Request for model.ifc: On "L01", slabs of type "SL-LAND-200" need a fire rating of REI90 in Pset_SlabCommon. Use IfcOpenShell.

First a look at what the model holds.

```python
import ifcopenshell
import ifcopenshell.util.element

model = ifcopenshell.open("model.ifc")
print(model.schema)
storey = next(s for s in model.by_type("IfcBuildingStorey") if s.Name == "L01")
slabs = [e for e in ifcopenshell.util.element.get_decomposition(storey) if e.is_a("IfcSlab")]
seen = {}
for e in slabs:
    element_type = ifcopenshell.util.element.get_type(e)
    key = (element_type.Name if element_type != e and element_type else None, ifcopenshell.util.element.get_pset(e, "Pset_SlabCommon", "FireRating"))
    seen[key] = seen.get(key, 0) + 1
for (name, value), count in sorted(seen.items(), key=str):
    print(count, "x", name, "|", value)
```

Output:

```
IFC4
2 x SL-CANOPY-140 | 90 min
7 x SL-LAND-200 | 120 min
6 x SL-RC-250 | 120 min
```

```python
import ifcopenshell
import ifcopenshell.api.pset
import ifcopenshell.util.element

model = ifcopenshell.open("model.ifc")

storey = next(s for s in model.by_type("IfcBuildingStorey") if s.Name == "L01")
slabs = [e for e in ifcopenshell.util.element.get_decomposition(storey) if e.is_a("IfcSlab")]

count = 0
for e in slabs:
    element_type = ifcopenshell.util.element.get_type(e)
    if element_type in (None, e) or element_type.Name != "SL-LAND-200":
        continue
    # add_pset returns the element's existing set when there is one.
    pset = ifcopenshell.api.pset.add_pset(model, product=e, name="Pset_SlabCommon")
    ifcopenshell.api.pset.edit_pset(model, pset=pset, properties={"FireRating": "REI90"})
    count += 1

print(count, "slabs updated")

model.write("model_v2.ifc")
```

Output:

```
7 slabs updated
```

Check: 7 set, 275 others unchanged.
